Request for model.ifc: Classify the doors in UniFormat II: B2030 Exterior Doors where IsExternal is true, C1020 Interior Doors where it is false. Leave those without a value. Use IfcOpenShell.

First a look at what the model holds.

```python
import ifcopenshell
import ifcopenshell.util.element

model = ifcopenshell.open("model.ifc")
print(model.schema)
print("classifications:", [c.Name for c in model.by_type("IfcClassification")])
values = [ifcopenshell.util.element.get_pset(e, "Pset_DoorCommon", "IsExternal") for e in model.by_type("IfcDoor")]
for value in (True, False, None):
    print("IsExternal", value, values.count(value))
```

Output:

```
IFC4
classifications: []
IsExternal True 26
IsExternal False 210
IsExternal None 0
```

```python
import ifcopenshell
import ifcopenshell.api.classification
import ifcopenshell.util.element

model = ifcopenshell.open("model.ifc")

system = ifcopenshell.api.classification.add_classification(model, classification="UniFormat II")

doors = model.by_type("IfcDoor")
external = {e: ifcopenshell.util.element.get_pset(e, "Pset_DoorCommon", "IsExternal") for e in doors}
for flag, code, name in ((True, "B2030", "Exterior Doors"), (False, "C1020", "Interior Doors")):
    products = [e for e in doors if external[e] is flag]
    ifcopenshell.api.classification.add_reference(
        model, products=products, classification=system, identification=code, name=name
    )
    print(code, len(products))

model.write("model_edited.ifc")
```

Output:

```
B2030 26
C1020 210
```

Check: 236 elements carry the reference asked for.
